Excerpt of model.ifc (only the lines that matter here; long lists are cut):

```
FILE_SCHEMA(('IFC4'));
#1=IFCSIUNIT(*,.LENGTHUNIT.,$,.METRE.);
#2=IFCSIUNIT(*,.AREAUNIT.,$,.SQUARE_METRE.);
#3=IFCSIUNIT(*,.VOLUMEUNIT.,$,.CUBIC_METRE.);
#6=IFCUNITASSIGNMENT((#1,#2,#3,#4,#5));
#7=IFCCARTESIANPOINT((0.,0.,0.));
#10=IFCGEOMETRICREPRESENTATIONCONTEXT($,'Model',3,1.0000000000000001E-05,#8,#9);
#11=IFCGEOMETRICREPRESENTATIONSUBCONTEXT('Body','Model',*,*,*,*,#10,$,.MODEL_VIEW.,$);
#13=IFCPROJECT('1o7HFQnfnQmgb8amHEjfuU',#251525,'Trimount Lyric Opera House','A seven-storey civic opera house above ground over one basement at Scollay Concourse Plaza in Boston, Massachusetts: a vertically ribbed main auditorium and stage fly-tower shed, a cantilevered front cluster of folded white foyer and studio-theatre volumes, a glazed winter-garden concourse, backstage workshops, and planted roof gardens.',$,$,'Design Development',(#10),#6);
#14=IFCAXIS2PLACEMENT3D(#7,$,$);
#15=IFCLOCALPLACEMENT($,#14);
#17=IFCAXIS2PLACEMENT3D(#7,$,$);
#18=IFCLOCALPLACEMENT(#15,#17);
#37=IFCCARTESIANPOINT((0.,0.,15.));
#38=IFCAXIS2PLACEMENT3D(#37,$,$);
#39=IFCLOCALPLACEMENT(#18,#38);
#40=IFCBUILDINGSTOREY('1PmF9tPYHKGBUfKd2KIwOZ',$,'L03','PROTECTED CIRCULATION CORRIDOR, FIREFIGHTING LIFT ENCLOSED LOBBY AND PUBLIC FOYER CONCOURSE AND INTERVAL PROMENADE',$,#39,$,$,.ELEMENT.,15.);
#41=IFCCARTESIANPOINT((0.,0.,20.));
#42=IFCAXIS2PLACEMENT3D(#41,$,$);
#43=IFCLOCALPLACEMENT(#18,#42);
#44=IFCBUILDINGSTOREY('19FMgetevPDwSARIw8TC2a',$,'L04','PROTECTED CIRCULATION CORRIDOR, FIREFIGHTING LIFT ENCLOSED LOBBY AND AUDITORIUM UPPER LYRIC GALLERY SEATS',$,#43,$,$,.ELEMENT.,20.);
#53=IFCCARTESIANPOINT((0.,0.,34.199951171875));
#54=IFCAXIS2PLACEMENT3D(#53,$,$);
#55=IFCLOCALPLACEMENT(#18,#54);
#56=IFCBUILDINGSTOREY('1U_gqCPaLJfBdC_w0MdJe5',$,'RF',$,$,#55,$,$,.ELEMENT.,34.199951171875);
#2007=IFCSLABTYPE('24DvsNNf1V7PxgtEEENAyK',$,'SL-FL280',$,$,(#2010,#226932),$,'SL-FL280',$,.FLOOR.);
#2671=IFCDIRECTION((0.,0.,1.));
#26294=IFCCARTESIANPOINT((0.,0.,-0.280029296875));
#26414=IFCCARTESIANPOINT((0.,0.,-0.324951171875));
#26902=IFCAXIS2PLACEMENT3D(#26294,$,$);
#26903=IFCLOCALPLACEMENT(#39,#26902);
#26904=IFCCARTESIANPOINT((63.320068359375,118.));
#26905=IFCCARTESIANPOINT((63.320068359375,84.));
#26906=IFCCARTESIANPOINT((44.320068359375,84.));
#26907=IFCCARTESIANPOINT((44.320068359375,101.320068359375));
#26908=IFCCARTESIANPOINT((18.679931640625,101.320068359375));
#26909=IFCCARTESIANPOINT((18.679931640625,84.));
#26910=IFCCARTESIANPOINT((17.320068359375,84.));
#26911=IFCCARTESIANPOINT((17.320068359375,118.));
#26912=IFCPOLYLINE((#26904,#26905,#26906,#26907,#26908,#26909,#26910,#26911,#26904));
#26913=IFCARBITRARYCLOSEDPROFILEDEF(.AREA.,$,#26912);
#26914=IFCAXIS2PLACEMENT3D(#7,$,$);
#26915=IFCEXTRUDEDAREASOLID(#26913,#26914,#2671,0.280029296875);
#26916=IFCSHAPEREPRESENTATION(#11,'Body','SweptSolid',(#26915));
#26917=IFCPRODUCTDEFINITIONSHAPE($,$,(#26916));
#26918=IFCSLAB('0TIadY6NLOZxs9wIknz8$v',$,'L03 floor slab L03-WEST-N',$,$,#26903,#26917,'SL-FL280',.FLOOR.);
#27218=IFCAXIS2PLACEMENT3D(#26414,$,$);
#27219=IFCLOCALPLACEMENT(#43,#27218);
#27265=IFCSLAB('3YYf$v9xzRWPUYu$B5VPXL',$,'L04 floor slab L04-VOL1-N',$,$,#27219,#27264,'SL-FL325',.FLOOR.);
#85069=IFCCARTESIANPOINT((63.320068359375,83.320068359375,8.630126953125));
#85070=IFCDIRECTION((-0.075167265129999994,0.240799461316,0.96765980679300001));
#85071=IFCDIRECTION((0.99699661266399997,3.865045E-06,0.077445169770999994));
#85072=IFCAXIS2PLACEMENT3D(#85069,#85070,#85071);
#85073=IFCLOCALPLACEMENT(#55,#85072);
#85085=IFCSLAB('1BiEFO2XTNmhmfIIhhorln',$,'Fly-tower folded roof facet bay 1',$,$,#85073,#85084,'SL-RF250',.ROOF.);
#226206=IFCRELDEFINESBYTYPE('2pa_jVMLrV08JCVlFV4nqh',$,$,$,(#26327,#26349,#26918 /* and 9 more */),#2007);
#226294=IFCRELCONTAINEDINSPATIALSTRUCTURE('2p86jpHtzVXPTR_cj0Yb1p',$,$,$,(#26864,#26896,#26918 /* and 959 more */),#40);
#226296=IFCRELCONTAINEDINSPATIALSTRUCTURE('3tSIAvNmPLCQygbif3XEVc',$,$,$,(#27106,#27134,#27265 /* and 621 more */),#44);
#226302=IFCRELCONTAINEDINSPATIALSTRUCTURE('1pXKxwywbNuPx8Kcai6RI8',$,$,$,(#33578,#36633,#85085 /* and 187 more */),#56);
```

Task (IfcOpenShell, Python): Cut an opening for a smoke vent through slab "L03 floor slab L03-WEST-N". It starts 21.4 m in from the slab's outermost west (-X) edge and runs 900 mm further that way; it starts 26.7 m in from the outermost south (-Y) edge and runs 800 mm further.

```python
import numpy as np
import ifcopenshell
import ifcopenshell.api.feature
import ifcopenshell.api.geometry
import ifcopenshell.api.root
import ifcopenshell.geom
import ifcopenshell.util.placement
import ifcopenshell.util.representation
import ifcopenshell.util.shape
import ifcopenshell.util.unit

model = ifcopenshell.open("model.ifc")
unit_scale = ifcopenshell.util.unit.calculate_unit_scale(model)
settings = ifcopenshell.geom.settings()


def volume(element):
    """Net volume in cubic metres, openings subtracted."""
    shape = ifcopenshell.geom.create_shape(settings, element)
    return ifcopenshell.util.shape.get_volume(shape.geometry)


slab = model.by_guid("0TIadY6NLOZxs9wIknz8$v")
before = volume(slab)

# Extent in the slab's own axes, in metres. The edges named are its -X and -Y sides.
slab_shape = ifcopenshell.geom.create_shape(settings, slab)
vertices = ifcopenshell.util.shape.get_vertices(slab_shape.geometry)
x_min, y_min, bottom = vertices.min(axis=0)
top = vertices[:, 2].max()

opening = ifcopenshell.api.root.create_entity(model, ifc_class="IfcOpeningElement", name="Smoke vent opening", predefined_type="OPENING")
context = ifcopenshell.util.representation.get_context(model, "Model", "Body", "MODEL_VIEW")
width, depth = 0.9, 0.8
outline = [(0.0, 0.0), (width, 0.0), (width, depth), (0.0, depth), (0.0, 0.0)]
# Overshoot both faces by 50 mm so the cut is clean.
shape = ifcopenshell.api.geometry.add_slab_representation(
    model, context=context, depth=top - bottom + 0.1, polyline=outline
)
ifcopenshell.api.geometry.assign_representation(model, product=opening, representation=shape)

matrix = ifcopenshell.util.placement.get_local_placement(slab.ObjectPlacement)
matrix[:, 3] = matrix @ np.append(np.array([x_min + 21.4, y_min + 26.7, bottom - 0.05]) / unit_scale, 1.0)
ifcopenshell.api.geometry.edit_object_placement(model, product=opening, matrix=matrix, is_si=False)
ifcopenshell.api.feature.add_feature(model, feature=opening, element=slab)

after = volume(slab)

print(f"slab volume {before:.3f} -> {after:.3f} m3")

model.write("model_edited.ifc")
```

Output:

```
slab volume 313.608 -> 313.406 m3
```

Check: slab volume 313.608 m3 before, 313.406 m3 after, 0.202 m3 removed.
